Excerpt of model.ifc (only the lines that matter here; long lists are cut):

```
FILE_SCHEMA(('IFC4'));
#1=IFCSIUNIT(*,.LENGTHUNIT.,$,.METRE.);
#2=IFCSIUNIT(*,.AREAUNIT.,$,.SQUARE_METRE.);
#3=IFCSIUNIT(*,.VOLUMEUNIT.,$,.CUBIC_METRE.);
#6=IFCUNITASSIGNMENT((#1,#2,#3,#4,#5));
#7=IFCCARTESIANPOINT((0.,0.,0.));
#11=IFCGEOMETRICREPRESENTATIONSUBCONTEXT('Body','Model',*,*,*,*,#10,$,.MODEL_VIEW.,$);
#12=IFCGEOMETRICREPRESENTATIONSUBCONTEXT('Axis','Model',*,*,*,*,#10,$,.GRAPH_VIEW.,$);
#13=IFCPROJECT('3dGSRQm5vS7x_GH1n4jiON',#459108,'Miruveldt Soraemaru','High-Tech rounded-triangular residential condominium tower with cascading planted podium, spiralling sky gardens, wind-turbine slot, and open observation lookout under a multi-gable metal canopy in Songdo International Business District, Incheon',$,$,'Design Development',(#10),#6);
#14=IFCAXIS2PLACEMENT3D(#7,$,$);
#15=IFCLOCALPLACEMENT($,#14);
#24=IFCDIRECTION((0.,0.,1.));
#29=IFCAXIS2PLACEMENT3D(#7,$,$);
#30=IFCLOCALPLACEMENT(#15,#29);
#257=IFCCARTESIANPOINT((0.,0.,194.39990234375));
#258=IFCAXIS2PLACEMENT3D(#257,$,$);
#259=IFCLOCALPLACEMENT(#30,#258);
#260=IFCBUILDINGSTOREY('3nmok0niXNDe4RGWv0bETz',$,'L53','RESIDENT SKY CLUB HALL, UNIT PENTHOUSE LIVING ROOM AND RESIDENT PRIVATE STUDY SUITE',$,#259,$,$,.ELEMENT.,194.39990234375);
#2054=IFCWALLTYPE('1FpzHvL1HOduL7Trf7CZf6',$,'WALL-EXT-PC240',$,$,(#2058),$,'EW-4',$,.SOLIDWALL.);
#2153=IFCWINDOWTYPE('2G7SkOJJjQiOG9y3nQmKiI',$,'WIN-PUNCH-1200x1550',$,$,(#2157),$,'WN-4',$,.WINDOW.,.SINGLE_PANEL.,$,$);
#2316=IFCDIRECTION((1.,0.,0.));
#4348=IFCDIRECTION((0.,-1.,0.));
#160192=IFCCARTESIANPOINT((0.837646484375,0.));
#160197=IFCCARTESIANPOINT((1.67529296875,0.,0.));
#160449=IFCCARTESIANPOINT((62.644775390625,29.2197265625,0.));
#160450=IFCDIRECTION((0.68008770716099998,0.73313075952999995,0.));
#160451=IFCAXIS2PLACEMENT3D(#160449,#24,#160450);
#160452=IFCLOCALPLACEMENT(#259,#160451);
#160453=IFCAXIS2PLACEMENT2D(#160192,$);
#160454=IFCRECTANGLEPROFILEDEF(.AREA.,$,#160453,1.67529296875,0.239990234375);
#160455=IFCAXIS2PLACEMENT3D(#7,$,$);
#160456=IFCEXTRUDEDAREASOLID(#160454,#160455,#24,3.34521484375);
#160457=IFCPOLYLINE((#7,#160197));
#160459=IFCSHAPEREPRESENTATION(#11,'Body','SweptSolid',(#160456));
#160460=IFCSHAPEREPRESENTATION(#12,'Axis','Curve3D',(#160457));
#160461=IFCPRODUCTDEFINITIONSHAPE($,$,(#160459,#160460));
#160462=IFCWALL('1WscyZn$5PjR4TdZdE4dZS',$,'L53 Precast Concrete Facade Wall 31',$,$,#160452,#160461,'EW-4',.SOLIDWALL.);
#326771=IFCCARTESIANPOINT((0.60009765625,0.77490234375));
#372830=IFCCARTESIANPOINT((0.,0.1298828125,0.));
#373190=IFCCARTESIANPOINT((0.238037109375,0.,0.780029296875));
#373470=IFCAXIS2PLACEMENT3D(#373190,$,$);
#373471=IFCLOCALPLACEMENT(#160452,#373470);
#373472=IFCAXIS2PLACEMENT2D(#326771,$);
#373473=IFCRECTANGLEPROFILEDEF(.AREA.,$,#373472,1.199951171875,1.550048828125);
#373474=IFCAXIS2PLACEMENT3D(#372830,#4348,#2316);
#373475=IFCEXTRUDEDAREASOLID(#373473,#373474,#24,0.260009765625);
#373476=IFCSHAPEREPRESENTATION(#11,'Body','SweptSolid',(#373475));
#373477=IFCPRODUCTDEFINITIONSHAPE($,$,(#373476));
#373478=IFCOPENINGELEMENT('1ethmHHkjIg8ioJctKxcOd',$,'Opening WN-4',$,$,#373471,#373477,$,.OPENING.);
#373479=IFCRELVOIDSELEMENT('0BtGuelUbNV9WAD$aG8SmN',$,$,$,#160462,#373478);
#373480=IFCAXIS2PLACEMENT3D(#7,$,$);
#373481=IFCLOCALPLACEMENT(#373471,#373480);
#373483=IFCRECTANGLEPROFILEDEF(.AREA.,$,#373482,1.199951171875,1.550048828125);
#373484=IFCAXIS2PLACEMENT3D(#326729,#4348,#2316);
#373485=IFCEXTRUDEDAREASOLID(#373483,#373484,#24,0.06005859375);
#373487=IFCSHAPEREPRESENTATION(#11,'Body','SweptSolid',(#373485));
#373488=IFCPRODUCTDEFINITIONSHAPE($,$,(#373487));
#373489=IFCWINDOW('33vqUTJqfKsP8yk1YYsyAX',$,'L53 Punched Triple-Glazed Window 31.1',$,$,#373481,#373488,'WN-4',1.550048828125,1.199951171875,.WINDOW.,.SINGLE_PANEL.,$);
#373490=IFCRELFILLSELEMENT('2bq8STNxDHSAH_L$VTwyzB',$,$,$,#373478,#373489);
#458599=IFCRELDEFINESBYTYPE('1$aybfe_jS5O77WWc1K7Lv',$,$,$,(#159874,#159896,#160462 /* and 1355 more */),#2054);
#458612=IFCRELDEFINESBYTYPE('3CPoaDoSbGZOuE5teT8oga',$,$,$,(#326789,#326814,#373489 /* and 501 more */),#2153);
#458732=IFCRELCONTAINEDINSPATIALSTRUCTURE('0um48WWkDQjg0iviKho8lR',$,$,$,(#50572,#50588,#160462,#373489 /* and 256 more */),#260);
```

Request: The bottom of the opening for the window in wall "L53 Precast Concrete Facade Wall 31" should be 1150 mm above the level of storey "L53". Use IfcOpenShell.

```python
import numpy as np
import ifcopenshell
import ifcopenshell.api.geometry
import ifcopenshell.geom
import ifcopenshell.util.element
import ifcopenshell.util.placement
import ifcopenshell.util.shape
import ifcopenshell.util.unit

model = ifcopenshell.open("model.ifc")
unit_scale = ifcopenshell.util.unit.calculate_unit_scale(model)

window = model.by_id(373489)
opening = window.FillsVoids[0].RelatingOpeningElement
storey = ifcopenshell.util.element.get_container(window, ifc_class="IfcBuildingStorey")
level = ifcopenshell.util.placement.get_local_placement(storey.ObjectPlacement)[2, 3]

# The opening's origin need not be at the sill, so measure its lowest point.
shape = ifcopenshell.geom.create_shape(ifcopenshell.geom.settings(), opening)
bottom = ifcopenshell.util.shape.get_shape_bottom_elevation(shape, shape.geometry) / unit_scale
dz = level + 1.15 / unit_scale - bottom

shift = np.array([0.0, 0.0, dz])
# The window is placed relative to its opening, so it follows when the opening moves.
matrix = ifcopenshell.util.placement.get_local_placement(opening.ObjectPlacement)
matrix[:3, 3] += shift
ifcopenshell.api.geometry.edit_object_placement(
    model, product=opening, matrix=matrix, is_si=False, should_transform_children=True
)

print(f"moved by {dz * unit_scale:+.3f} m")

model.write("model_v2.ifc")
```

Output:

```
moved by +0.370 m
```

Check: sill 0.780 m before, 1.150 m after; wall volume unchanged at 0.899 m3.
